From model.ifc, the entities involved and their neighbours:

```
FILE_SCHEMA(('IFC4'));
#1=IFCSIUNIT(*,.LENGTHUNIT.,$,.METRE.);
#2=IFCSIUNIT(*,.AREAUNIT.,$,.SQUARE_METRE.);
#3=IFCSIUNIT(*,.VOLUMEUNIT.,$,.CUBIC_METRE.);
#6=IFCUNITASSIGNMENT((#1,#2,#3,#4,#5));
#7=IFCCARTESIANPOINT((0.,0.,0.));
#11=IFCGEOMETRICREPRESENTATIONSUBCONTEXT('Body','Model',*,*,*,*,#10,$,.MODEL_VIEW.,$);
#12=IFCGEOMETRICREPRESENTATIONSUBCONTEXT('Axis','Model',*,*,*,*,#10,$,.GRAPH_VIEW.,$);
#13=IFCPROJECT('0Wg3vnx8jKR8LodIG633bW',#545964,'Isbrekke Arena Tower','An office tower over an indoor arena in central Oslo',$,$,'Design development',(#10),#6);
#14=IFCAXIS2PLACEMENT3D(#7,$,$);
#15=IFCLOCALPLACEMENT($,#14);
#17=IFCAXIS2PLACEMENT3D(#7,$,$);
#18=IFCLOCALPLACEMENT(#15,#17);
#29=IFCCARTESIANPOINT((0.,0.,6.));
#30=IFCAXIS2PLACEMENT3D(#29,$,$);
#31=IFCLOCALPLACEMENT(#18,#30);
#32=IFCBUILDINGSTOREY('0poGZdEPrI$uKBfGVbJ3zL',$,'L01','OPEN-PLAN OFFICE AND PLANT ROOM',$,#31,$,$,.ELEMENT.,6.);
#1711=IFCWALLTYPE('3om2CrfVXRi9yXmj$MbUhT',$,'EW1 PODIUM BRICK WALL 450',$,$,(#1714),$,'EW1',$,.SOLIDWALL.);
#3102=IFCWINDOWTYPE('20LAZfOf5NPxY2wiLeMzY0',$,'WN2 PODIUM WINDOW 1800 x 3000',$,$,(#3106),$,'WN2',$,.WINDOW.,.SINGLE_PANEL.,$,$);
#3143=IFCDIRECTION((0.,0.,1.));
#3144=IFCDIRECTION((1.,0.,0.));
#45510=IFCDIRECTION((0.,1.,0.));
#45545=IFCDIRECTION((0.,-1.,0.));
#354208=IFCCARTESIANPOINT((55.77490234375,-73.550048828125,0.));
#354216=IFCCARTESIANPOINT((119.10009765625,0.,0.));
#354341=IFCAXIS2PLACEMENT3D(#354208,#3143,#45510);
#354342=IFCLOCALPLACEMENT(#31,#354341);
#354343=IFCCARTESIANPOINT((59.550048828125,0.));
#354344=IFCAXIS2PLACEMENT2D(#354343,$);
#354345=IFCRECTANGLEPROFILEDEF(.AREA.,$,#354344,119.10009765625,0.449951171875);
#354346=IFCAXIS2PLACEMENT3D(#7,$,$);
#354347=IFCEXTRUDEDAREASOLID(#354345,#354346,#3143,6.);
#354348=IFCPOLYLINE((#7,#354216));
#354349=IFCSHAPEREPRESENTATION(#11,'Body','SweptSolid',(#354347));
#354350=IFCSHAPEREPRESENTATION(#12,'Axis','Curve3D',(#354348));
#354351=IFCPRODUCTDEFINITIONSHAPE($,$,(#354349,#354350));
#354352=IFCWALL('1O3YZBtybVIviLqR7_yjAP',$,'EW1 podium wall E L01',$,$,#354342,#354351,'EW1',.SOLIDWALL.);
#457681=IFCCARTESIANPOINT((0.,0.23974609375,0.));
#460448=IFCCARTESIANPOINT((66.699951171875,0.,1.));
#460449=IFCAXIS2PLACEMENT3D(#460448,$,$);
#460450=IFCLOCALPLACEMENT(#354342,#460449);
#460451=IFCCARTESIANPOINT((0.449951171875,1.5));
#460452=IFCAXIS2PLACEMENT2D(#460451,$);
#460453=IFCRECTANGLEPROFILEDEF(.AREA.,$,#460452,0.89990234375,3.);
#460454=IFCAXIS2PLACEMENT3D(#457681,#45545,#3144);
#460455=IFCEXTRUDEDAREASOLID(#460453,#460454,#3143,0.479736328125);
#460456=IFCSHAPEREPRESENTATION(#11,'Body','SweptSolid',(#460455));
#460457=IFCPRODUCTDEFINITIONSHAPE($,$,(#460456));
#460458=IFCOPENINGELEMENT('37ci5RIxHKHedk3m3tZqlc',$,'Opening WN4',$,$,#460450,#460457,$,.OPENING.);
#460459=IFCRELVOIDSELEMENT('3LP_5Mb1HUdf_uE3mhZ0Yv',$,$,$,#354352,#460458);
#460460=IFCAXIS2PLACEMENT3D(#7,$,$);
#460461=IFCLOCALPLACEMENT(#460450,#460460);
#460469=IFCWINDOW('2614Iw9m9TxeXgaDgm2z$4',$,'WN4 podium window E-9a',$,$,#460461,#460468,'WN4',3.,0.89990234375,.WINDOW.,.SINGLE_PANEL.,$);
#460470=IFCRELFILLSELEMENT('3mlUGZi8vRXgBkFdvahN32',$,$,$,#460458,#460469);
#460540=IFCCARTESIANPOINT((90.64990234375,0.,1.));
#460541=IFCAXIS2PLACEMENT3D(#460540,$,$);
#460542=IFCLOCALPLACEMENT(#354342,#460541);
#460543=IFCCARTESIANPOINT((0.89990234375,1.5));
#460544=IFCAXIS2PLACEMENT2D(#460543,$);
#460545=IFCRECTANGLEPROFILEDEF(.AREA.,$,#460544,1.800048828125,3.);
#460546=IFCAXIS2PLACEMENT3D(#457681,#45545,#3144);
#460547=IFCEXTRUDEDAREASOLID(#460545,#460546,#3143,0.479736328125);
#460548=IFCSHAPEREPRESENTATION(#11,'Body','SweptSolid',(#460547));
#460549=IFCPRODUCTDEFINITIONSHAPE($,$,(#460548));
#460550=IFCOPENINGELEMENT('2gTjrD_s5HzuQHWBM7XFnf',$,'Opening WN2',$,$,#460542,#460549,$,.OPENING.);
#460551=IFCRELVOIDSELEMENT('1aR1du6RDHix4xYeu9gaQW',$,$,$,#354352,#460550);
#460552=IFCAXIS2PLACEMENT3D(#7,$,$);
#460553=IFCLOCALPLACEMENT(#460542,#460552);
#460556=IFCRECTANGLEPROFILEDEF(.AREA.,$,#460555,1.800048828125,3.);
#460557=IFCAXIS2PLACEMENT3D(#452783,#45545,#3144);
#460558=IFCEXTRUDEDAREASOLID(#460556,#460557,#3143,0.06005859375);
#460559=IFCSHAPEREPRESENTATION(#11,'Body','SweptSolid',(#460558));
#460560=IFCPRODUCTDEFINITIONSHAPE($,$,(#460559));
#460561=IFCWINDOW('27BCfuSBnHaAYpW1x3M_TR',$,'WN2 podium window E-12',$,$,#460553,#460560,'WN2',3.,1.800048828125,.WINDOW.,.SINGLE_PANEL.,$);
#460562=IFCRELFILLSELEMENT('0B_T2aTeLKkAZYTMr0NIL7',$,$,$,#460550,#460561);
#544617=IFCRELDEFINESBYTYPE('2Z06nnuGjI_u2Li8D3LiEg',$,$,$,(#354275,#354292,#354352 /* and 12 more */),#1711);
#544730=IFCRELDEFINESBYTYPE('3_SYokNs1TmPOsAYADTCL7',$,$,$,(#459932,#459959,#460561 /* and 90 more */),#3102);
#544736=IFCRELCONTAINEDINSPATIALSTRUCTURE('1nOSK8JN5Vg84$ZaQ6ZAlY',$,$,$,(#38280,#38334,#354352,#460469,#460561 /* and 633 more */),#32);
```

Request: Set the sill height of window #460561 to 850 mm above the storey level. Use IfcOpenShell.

```python
import numpy as np
import ifcopenshell
import ifcopenshell.api.geometry
import ifcopenshell.geom
import ifcopenshell.util.element
import ifcopenshell.util.placement
import ifcopenshell.util.shape
import ifcopenshell.util.unit

model = ifcopenshell.open("model.ifc")
unit_scale = ifcopenshell.util.unit.calculate_unit_scale(model)

window = model.by_guid("27BCfuSBnHaAYpW1x3M_TR")
opening = window.FillsVoids[0].RelatingOpeningElement
storey = ifcopenshell.util.element.get_container(window, ifc_class="IfcBuildingStorey")
level = ifcopenshell.util.placement.get_local_placement(storey.ObjectPlacement)[2, 3]

# The opening's origin need not be at the sill, so measure its lowest point.
shape = ifcopenshell.geom.create_shape(ifcopenshell.geom.settings(), opening)
bottom = ifcopenshell.util.shape.get_shape_bottom_elevation(shape, shape.geometry) / unit_scale
dz = level + 0.85 / unit_scale - bottom

shift = np.array([0.0, 0.0, dz])
# The window is placed relative to its opening, so it follows when the opening moves.
matrix = ifcopenshell.util.placement.get_local_placement(opening.ObjectPlacement)
matrix[:3, 3] += shift
ifcopenshell.api.geometry.edit_object_placement(
    model, product=opening, matrix=matrix, is_si=False, should_transform_children=True
)

print(f"moved by {dz * unit_scale:+.3f} m")

model.write("model_rev.ifc")
```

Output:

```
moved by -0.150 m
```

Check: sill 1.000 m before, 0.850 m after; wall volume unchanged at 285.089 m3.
